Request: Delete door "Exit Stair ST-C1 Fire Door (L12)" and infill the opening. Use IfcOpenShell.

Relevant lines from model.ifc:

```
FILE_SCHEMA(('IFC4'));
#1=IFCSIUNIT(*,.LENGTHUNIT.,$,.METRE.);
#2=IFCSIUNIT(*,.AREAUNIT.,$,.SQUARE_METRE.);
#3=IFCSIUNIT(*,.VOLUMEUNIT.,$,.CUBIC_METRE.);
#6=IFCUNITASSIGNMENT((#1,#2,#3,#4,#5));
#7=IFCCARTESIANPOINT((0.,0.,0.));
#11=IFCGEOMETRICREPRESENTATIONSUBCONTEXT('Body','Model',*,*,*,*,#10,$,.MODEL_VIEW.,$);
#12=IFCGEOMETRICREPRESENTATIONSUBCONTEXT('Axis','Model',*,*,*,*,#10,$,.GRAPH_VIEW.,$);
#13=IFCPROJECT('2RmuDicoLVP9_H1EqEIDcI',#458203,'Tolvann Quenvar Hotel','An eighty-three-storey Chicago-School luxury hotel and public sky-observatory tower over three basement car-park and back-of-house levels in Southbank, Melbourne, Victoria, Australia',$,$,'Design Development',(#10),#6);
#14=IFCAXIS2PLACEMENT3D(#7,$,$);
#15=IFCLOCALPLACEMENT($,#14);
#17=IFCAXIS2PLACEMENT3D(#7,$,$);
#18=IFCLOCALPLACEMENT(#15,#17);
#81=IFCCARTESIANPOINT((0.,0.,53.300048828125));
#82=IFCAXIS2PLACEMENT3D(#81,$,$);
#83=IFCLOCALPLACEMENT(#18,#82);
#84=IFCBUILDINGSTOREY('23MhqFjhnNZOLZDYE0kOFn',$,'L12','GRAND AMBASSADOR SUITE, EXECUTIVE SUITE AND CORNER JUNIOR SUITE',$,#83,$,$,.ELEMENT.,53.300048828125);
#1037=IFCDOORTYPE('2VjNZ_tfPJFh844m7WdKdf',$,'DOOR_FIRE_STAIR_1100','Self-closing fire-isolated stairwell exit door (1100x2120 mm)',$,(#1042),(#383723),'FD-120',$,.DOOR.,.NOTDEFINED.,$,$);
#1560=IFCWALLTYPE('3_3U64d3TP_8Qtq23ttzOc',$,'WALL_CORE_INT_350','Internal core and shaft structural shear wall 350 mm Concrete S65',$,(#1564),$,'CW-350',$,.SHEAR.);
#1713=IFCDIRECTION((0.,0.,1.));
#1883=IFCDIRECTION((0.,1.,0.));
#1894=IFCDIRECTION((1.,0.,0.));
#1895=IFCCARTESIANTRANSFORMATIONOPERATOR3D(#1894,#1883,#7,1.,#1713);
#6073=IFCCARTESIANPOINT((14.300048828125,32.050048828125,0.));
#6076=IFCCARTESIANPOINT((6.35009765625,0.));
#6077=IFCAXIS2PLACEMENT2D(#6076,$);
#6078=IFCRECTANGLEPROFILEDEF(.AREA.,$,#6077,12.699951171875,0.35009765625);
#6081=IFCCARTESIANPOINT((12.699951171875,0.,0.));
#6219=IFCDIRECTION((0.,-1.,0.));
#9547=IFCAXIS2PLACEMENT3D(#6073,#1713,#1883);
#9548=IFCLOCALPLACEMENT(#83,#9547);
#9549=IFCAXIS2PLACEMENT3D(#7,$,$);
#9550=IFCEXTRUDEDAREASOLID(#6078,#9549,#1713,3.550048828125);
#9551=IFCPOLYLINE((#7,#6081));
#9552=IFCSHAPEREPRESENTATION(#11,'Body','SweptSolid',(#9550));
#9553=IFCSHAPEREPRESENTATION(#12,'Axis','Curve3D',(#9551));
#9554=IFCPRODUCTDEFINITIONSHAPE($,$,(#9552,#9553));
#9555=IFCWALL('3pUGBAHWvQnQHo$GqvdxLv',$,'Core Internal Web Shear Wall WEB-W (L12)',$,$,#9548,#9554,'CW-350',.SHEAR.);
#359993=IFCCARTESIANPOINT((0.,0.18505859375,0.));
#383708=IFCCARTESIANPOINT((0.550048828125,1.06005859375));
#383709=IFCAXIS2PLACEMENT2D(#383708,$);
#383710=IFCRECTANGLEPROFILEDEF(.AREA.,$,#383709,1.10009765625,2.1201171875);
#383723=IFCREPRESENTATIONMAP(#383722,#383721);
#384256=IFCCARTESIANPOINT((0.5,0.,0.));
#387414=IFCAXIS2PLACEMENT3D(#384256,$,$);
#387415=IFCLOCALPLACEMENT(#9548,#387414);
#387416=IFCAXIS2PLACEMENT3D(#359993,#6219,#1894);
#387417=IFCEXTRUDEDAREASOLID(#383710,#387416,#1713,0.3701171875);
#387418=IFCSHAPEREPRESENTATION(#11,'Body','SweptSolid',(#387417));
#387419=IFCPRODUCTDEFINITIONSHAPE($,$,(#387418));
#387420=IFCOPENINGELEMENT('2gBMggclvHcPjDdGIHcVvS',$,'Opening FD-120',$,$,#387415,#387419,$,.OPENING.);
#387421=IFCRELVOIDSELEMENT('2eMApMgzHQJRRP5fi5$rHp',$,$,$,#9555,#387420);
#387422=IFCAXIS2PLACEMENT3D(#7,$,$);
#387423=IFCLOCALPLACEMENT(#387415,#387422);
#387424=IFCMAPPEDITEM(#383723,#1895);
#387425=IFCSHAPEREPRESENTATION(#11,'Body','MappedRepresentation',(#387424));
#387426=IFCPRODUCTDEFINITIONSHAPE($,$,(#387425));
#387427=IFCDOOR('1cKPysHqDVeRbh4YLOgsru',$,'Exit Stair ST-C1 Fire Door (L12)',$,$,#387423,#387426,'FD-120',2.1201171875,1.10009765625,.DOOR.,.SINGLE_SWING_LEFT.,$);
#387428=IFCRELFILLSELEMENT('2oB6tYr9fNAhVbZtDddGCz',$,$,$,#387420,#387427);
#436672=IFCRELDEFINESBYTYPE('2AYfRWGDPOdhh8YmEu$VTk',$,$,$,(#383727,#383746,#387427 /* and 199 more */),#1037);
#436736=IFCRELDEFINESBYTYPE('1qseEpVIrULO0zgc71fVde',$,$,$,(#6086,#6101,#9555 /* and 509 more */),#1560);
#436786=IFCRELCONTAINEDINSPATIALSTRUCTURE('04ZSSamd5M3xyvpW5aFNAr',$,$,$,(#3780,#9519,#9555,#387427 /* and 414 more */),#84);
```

```python
import ifcopenshell
import ifcopenshell.api.feature
import ifcopenshell.api.root
import ifcopenshell.geom
import ifcopenshell.util.shape

model = ifcopenshell.open("model.ifc")
settings = ifcopenshell.geom.settings()


def volume(element):
    """Net volume in cubic metres, openings subtracted."""
    shape = ifcopenshell.geom.create_shape(settings, element)
    return ifcopenshell.util.shape.get_volume(shape.geometry)


door = model.by_guid("1cKPysHqDVeRbh4YLOgsru")
opening = door.FillsVoids[0].RelatingOpeningElement
wall = opening.VoidsElements[0].RelatingBuildingElement
before = volume(wall)

ifcopenshell.api.root.remove_product(model, product=door)
ifcopenshell.api.feature.remove_feature(model, feature=opening)

after = volume(wall)

print(f"wall volume {before:.3f} -> {after:.3f} m3")

model.write("model_rev.ifc")
```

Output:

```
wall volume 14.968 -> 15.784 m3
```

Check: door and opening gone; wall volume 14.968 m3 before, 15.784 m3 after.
